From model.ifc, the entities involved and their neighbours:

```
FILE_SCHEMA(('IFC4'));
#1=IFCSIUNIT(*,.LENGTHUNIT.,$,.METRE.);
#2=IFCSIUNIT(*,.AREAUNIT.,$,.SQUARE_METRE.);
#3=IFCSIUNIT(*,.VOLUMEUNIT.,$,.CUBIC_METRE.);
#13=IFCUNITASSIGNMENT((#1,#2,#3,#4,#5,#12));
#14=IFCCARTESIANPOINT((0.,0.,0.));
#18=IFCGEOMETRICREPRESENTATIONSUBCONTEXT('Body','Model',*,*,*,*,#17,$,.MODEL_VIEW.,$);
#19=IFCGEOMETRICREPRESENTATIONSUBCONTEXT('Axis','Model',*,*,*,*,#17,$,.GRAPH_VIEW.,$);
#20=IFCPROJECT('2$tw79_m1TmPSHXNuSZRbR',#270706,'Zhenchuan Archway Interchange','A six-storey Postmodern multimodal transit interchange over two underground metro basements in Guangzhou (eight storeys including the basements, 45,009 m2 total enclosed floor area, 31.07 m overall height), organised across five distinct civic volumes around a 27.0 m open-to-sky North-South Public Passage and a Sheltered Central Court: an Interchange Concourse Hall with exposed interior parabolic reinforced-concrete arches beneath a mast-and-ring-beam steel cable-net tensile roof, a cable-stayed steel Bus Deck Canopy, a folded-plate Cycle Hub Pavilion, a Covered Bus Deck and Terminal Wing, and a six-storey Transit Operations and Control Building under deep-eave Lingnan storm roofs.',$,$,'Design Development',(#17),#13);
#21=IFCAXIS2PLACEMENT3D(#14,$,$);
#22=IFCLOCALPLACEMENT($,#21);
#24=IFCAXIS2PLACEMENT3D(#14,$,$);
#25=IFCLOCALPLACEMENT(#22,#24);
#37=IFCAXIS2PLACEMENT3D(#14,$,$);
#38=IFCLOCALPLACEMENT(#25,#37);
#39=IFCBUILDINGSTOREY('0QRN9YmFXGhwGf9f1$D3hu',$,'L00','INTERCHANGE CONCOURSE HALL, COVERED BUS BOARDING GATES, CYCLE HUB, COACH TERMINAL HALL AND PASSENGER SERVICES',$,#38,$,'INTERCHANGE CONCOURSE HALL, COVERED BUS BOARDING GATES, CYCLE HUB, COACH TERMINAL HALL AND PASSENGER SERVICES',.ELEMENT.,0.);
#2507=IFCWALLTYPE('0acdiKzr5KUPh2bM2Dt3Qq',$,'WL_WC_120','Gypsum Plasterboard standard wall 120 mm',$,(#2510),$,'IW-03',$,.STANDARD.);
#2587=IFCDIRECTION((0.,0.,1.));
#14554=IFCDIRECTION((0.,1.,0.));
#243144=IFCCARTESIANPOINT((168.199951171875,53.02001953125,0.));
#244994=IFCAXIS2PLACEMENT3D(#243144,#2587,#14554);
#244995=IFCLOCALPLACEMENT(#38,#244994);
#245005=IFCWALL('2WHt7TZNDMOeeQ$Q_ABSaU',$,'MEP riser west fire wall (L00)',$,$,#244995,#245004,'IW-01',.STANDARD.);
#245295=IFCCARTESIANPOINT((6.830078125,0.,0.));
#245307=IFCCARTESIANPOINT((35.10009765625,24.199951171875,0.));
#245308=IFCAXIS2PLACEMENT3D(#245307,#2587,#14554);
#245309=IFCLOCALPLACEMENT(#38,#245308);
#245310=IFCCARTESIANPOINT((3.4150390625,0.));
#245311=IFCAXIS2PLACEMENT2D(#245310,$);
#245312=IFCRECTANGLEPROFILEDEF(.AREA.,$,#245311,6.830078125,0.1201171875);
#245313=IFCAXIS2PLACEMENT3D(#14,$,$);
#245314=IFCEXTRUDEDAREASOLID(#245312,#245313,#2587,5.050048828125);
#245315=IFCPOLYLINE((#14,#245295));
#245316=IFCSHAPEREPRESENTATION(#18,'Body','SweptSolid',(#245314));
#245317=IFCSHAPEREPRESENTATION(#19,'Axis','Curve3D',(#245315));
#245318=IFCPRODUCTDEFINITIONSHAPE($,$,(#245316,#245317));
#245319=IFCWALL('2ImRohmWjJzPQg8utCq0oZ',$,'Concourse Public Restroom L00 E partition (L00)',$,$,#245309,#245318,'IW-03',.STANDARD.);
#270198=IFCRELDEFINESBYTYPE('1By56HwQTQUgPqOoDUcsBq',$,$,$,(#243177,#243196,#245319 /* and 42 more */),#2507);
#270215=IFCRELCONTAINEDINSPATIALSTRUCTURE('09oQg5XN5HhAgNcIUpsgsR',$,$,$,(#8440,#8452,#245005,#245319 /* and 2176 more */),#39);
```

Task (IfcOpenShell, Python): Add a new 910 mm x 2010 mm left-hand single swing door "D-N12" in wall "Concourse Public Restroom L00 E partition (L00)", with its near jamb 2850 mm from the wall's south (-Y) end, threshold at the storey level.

```python
import numpy as np
import ifcopenshell
import ifcopenshell.api.feature
import ifcopenshell.api.geometry
import ifcopenshell.api.root
import ifcopenshell.api.spatial
import ifcopenshell.geom
import ifcopenshell.util.element
import ifcopenshell.util.placement
import ifcopenshell.util.representation
import ifcopenshell.util.shape
import ifcopenshell.util.unit

model = ifcopenshell.open("model.ifc")
unit_scale = ifcopenshell.util.unit.calculate_unit_scale(model)
settings = ifcopenshell.geom.settings()


def volume(element):
    """Net volume in cubic metres, openings subtracted."""
    shape = ifcopenshell.geom.create_shape(settings, element)
    return ifcopenshell.util.shape.get_volume(shape.geometry)


wall = model.by_guid("2ImRohmWjJzPQg8utCq0oZ")
storey = ifcopenshell.util.element.get_container(wall, ifc_class="IfcBuildingStorey")
context = ifcopenshell.util.representation.get_context(model, "Model", "Body", "MODEL_VIEW")
before = volume(wall)

width, height, from_end, sill = 0.91, 2.01, 2.85, 0.0  # metres

# The wall runs along its own X axis, and the end named is its -X end.
wall_shape = ifcopenshell.geom.create_shape(settings, wall)
x, y, z = ifcopenshell.util.shape.get_vertices(wall_shape.geometry).T
start = x.min() + from_end
face, thickness = float(y.min()), float(y.max() - y.min())
wall_matrix = ifcopenshell.util.placement.get_local_placement(wall.ObjectPlacement)
level = ifcopenshell.util.placement.get_local_placement(storey.ObjectPlacement)[2, 3]


def in_wall(x, y):
    """Placement at x, y metres in the wall's axes, at sill height."""
    matrix = wall_matrix.copy()
    matrix[:, 3] = wall_matrix @ np.array([x / unit_scale, y / unit_scale, 0.0, 1.0])
    matrix[2, 3] = level + sill / unit_scale
    return matrix


# Opening: a box that overshoots both wall faces by 50 mm.
opening = ifcopenshell.api.root.create_entity(model, ifc_class="IfcOpeningElement", predefined_type="OPENING")
box = ifcopenshell.api.geometry.add_wall_representation(
    model, context=context, length=width, height=height, thickness=thickness + 0.1
)
ifcopenshell.api.geometry.assign_representation(model, product=opening, representation=box)
ifcopenshell.api.geometry.edit_object_placement(model, product=opening, matrix=in_wall(start, face - 0.05), is_si=False)
ifcopenshell.api.feature.add_feature(model, feature=opening, element=wall)

door = ifcopenshell.api.root.create_entity(model, ifc_class="IfcDoor", name="D-N12", predefined_type="DOOR")
door.OverallWidth, door.OverallHeight = width / unit_scale, height / unit_scale
door.OperationType = "SINGLE_SWING_LEFT"
body = ifcopenshell.api.geometry.add_door_representation(
    model,
    context=context,
    overall_width=door.OverallWidth,
    overall_height=door.OverallHeight,
    operation_type="SINGLE_SWING_LEFT",
    lining_properties={"LiningDepth": thickness / unit_scale, "ThresholdDepth": thickness / unit_scale},
)
ifcopenshell.api.geometry.assign_representation(model, product=door, representation=body)
ifcopenshell.api.spatial.assign_container(model, products=[door], relating_structure=storey)
ifcopenshell.api.feature.add_filling(model, opening=opening, element=door)

# The lining spans the wall, so the door starts at the wall face.
ifcopenshell.api.geometry.edit_object_placement(model, product=door, matrix=in_wall(start, face), is_si=False)

after = volume(wall)

print(f"wall volume {before:.3f} -> {after:.3f} m3")

model.write("model_edited.ifc")
```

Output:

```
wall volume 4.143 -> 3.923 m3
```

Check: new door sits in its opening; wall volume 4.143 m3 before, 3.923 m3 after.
